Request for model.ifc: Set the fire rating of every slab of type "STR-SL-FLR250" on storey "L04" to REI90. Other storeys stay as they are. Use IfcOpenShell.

First a look at what the model holds.

```python
import ifcopenshell
import ifcopenshell.util.element

model = ifcopenshell.open("model.ifc")
print(model.schema)
storey = next(s for s in model.by_type("IfcBuildingStorey") if s.Name == "L04")
slabs = [e for e in ifcopenshell.util.element.get_decomposition(storey) if e.is_a("IfcSlab")]
seen = {}
for e in slabs:
    element_type = ifcopenshell.util.element.get_type(e)
    key = (element_type.Name if element_type != e and element_type else None, ifcopenshell.util.element.get_pset(e, "Pset_SlabCommon", "FireRating"))
    seen[key] = seen.get(key, 0) + 1
for (name, value), count in sorted(seen.items(), key=str):
    print(count, "x", name, "|", value)
```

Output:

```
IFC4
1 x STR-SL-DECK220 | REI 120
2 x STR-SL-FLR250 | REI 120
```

```python
import ifcopenshell
import ifcopenshell.api.pset
import ifcopenshell.util.element

model = ifcopenshell.open("model.ifc")

storey = next(s for s in model.by_type("IfcBuildingStorey") if s.Name == "L04")
slabs = [e for e in ifcopenshell.util.element.get_decomposition(storey) if e.is_a("IfcSlab")]

count = 0
for e in slabs:
    element_type = ifcopenshell.util.element.get_type(e)
    if element_type in (None, e) or element_type.Name != "STR-SL-FLR250":
        continue
    # add_pset returns the element's existing set when there is one.
    pset = ifcopenshell.api.pset.add_pset(model, product=e, name="Pset_SlabCommon")
    ifcopenshell.api.pset.edit_pset(model, pset=pset, properties={"FireRating": "REI90"})
    count += 1

print(count, "slabs updated")

model.write("model_updated.ifc")
```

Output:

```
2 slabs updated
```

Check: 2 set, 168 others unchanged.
